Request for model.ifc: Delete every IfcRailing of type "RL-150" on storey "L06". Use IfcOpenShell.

First a look at what the model holds.

```python
import ifcopenshell
import ifcopenshell.util.element

model = ifcopenshell.open("model.ifc")
print(model.schema)
storey = next(s for s in model.by_type("IfcBuildingStorey") if s.Name == "L06")
railings = [e for e in ifcopenshell.util.element.get_decomposition(storey) if e.is_a("IfcRailing")]
seen = {}
for e in railings:
    element_type = ifcopenshell.util.element.get_type(e)
    name = element_type.Name if element_type not in (None, e) else None
    seen[name] = seen.get(name, 0) + 1
for name, count in sorted(seen.items(), key=str):
    print(count, "x", name)
```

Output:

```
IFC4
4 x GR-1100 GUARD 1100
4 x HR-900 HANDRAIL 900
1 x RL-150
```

```python
import ifcopenshell
import ifcopenshell.api.root
import ifcopenshell.util.element

model = ifcopenshell.open("model.ifc")

storey = next(s for s in model.by_type("IfcBuildingStorey") if s.Name == "L06")
railings = [e for e in ifcopenshell.util.element.get_decomposition(storey) if e.is_a("IfcRailing")]
targets = [e for e in railings if (t := ifcopenshell.util.element.get_type(e)) not in (None, e) and t.Name == "RL-150"]

for e in targets:
    ifcopenshell.api.root.remove_product(model, product=e)
print(len(targets), "removed")

model.write("model-out.ifc")
```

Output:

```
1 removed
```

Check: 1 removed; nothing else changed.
